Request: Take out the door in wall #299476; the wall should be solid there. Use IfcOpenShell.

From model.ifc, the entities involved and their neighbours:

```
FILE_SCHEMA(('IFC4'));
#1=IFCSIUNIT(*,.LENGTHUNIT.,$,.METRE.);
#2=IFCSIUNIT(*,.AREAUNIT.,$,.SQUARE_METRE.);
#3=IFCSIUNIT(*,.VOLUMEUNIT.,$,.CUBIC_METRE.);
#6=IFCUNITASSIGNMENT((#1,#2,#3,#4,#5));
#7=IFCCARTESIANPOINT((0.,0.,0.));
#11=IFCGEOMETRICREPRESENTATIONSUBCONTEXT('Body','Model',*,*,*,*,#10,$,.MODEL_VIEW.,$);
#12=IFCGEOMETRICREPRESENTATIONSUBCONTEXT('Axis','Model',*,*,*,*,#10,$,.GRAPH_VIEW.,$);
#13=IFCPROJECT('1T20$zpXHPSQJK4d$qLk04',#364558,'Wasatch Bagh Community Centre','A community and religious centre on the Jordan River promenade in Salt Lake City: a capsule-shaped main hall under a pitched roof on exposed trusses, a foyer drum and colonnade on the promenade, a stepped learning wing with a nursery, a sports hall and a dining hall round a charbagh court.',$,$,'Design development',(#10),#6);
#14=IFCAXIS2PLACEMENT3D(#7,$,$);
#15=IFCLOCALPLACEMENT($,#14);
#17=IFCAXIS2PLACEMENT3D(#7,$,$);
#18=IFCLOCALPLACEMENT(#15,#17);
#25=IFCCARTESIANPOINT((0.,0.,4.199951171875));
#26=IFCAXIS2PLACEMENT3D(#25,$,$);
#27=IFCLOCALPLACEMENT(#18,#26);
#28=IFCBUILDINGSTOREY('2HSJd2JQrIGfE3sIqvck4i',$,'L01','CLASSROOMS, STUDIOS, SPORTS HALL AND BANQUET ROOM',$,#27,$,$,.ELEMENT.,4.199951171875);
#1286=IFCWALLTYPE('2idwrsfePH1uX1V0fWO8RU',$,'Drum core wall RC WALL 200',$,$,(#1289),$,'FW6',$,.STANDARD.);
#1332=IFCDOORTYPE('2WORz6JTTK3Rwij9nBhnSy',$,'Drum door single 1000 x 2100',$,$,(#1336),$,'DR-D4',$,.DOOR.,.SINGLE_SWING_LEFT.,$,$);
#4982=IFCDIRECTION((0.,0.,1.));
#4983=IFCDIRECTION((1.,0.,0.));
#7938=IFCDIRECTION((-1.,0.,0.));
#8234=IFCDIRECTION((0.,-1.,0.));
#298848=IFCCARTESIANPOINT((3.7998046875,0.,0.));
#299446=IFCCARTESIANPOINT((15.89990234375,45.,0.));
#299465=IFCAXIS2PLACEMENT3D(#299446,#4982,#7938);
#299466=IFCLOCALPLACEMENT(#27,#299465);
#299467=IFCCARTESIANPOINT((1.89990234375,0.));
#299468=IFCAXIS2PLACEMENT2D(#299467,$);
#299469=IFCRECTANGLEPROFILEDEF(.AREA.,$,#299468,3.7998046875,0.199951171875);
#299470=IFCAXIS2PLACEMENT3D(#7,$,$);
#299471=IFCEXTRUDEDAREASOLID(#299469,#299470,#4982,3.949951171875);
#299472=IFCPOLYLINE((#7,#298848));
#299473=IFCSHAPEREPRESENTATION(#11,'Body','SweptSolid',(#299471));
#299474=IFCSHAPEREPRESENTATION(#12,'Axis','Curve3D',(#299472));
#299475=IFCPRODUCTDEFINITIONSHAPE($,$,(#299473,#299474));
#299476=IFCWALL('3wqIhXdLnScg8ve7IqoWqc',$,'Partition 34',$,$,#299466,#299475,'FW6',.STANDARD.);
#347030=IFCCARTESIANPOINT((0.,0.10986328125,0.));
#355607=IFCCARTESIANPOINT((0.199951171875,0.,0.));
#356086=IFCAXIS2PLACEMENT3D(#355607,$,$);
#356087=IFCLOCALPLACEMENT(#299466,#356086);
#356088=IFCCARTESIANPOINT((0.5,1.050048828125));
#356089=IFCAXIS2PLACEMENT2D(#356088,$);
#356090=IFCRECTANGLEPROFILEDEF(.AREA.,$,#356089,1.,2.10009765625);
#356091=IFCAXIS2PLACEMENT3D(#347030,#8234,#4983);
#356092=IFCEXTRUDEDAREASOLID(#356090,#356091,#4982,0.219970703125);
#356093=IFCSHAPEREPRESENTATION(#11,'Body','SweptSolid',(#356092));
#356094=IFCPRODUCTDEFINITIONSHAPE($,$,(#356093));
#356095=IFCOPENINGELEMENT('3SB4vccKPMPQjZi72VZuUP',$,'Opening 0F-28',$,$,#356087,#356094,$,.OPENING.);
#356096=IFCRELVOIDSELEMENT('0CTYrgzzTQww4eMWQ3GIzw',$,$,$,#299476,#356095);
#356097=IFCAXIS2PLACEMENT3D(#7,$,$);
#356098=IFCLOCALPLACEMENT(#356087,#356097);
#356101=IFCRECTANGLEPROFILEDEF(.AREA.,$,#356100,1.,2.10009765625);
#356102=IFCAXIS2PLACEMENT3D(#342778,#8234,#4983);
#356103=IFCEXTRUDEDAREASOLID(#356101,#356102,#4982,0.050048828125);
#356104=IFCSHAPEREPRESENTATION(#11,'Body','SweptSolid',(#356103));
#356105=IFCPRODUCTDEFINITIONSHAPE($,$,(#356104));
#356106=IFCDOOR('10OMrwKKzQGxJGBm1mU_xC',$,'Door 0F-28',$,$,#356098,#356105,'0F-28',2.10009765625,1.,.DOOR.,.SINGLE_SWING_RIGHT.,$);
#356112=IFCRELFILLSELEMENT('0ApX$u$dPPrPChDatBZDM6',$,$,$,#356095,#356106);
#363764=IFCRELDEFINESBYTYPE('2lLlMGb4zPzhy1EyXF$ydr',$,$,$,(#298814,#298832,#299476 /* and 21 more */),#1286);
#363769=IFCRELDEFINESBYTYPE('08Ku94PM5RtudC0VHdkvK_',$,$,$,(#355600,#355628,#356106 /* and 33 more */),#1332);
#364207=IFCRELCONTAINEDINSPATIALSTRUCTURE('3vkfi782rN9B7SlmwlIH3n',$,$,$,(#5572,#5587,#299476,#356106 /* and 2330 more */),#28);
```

```python
import ifcopenshell
import ifcopenshell.api.feature
import ifcopenshell.api.root
import ifcopenshell.geom
import ifcopenshell.util.shape

model = ifcopenshell.open("model.ifc")
settings = ifcopenshell.geom.settings()


def volume(element):
    """Net volume in cubic metres, openings subtracted."""
    shape = ifcopenshell.geom.create_shape(settings, element)
    return ifcopenshell.util.shape.get_volume(shape.geometry)


door = model.by_id(356106)
opening = door.FillsVoids[0].RelatingOpeningElement
wall = opening.VoidsElements[0].RelatingBuildingElement
before = volume(wall)

ifcopenshell.api.root.remove_product(model, product=door)
ifcopenshell.api.feature.remove_feature(model, feature=opening)

after = volume(wall)

print(f"wall volume {before:.3f} -> {after:.3f} m3")

model.write("model_v2.ifc")
```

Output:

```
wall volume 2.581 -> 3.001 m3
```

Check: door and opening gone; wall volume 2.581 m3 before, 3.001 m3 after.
